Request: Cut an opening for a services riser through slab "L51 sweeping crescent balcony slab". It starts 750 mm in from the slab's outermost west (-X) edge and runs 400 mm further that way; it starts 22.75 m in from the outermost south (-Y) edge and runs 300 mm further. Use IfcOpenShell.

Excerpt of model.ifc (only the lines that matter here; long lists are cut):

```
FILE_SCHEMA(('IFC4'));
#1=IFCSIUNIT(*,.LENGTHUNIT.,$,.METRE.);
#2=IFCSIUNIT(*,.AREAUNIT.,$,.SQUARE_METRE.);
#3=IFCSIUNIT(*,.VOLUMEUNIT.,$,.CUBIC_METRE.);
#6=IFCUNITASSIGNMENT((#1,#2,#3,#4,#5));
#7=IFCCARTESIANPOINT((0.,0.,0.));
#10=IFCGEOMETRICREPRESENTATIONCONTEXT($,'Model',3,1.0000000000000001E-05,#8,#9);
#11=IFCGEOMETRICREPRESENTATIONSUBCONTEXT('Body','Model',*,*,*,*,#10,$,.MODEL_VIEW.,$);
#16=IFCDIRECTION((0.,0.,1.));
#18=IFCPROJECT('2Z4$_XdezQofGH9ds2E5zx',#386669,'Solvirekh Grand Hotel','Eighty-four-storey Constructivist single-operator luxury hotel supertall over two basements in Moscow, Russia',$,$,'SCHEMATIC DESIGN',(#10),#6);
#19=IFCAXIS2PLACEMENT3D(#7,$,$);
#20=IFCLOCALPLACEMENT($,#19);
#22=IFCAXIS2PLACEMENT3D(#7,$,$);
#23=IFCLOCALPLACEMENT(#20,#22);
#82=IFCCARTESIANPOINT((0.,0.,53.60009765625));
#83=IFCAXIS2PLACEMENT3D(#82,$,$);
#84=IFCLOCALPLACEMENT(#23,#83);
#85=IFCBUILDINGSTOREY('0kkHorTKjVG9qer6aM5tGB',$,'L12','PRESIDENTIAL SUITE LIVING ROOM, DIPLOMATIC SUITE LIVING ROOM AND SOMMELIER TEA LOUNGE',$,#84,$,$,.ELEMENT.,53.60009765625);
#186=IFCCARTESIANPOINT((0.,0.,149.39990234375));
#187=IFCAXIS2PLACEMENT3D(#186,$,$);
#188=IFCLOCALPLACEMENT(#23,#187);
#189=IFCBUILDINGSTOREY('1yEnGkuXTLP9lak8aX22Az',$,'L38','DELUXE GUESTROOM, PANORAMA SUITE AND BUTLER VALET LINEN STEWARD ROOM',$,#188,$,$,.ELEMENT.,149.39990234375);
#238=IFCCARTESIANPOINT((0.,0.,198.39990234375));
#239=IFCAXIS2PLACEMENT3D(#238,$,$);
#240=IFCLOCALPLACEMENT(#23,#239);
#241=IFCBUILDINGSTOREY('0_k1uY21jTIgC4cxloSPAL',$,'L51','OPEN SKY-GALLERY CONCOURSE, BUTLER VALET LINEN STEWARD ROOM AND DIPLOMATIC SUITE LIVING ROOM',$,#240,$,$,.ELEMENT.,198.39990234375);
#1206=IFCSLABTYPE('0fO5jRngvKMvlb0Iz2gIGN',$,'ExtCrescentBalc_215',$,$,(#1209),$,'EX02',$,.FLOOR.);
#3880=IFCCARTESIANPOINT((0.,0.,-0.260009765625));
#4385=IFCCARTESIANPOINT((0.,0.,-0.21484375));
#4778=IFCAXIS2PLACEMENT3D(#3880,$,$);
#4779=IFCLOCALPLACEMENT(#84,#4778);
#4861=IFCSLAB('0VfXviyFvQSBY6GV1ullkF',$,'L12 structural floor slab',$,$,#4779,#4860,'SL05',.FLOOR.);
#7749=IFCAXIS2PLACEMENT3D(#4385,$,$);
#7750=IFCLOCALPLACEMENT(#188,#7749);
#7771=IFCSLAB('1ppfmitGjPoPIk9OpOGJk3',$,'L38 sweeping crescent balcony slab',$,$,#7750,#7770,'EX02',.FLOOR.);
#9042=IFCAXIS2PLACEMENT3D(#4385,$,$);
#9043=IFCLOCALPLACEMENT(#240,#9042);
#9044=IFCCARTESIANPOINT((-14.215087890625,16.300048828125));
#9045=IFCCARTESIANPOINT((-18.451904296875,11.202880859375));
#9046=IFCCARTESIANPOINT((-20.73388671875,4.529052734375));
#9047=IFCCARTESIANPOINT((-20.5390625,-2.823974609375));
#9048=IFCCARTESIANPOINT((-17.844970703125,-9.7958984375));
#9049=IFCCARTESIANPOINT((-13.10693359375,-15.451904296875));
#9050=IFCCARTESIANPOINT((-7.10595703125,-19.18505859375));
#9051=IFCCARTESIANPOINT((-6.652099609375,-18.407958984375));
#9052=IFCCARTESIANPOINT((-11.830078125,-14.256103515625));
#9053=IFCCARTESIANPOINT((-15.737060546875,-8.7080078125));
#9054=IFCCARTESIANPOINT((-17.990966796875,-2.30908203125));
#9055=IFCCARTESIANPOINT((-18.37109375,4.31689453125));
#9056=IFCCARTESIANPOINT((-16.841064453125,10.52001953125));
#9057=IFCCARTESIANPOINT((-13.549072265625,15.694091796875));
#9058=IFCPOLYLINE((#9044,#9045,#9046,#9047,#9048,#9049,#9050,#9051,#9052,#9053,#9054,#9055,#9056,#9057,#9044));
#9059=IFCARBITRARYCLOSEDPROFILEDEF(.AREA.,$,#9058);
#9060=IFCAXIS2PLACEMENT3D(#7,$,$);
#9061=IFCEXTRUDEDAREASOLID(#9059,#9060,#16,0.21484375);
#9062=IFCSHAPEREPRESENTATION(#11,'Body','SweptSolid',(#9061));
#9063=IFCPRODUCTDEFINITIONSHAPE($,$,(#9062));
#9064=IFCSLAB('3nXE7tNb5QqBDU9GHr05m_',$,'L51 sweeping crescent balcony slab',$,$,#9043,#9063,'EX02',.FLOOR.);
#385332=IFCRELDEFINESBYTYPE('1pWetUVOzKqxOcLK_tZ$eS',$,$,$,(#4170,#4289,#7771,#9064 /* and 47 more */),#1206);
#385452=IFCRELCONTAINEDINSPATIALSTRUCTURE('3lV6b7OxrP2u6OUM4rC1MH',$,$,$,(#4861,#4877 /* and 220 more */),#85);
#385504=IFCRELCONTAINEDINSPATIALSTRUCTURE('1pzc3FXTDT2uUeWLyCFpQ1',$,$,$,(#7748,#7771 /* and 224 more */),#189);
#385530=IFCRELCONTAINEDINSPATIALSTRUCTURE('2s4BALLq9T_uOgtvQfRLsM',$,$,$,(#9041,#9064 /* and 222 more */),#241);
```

```python
import numpy as np
import ifcopenshell
import ifcopenshell.api.feature
import ifcopenshell.api.geometry
import ifcopenshell.api.root
import ifcopenshell.geom
import ifcopenshell.util.placement
import ifcopenshell.util.representation
import ifcopenshell.util.shape
import ifcopenshell.util.unit

model = ifcopenshell.open("model.ifc")
unit_scale = ifcopenshell.util.unit.calculate_unit_scale(model)
settings = ifcopenshell.geom.settings()


def volume(element):
    """Net volume in cubic metres, openings subtracted."""
    shape = ifcopenshell.geom.create_shape(settings, element)
    return ifcopenshell.util.shape.get_volume(shape.geometry)


slab = model.by_guid("3nXE7tNb5QqBDU9GHr05m_")
before = volume(slab)

# Extent in the slab's own axes, in metres. The edges named are its -X and -Y sides.
slab_shape = ifcopenshell.geom.create_shape(settings, slab)
vertices = ifcopenshell.util.shape.get_vertices(slab_shape.geometry)
x_min, y_min, bottom = vertices.min(axis=0)
top = vertices[:, 2].max()

opening = ifcopenshell.api.root.create_entity(model, ifc_class="IfcOpeningElement", name="Services riser opening", predefined_type="OPENING")
context = ifcopenshell.util.representation.get_context(model, "Model", "Body", "MODEL_VIEW")
width, depth = 0.4, 0.3
outline = [(0.0, 0.0), (width, 0.0), (width, depth), (0.0, depth), (0.0, 0.0)]
# Overshoot both faces by 50 mm so the cut is clean.
shape = ifcopenshell.api.geometry.add_slab_representation(
    model, context=context, depth=top - bottom + 0.1, polyline=outline
)
ifcopenshell.api.geometry.assign_representation(model, product=opening, representation=shape)

matrix = ifcopenshell.util.placement.get_local_placement(slab.ObjectPlacement)
matrix[:, 3] = matrix @ np.append(np.array([x_min + 0.75, y_min + 22.75, bottom - 0.05]) / unit_scale, 1.0)
ifcopenshell.api.geometry.edit_object_placement(model, product=opening, matrix=matrix, is_si=False)
ifcopenshell.api.feature.add_feature(model, feature=opening, element=slab)

after = volume(slab)

print(f"slab volume {before:.3f} -> {after:.3f} m3")

model.write("model_updated.ifc")
```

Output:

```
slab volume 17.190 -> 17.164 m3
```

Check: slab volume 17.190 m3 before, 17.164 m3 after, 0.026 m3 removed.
